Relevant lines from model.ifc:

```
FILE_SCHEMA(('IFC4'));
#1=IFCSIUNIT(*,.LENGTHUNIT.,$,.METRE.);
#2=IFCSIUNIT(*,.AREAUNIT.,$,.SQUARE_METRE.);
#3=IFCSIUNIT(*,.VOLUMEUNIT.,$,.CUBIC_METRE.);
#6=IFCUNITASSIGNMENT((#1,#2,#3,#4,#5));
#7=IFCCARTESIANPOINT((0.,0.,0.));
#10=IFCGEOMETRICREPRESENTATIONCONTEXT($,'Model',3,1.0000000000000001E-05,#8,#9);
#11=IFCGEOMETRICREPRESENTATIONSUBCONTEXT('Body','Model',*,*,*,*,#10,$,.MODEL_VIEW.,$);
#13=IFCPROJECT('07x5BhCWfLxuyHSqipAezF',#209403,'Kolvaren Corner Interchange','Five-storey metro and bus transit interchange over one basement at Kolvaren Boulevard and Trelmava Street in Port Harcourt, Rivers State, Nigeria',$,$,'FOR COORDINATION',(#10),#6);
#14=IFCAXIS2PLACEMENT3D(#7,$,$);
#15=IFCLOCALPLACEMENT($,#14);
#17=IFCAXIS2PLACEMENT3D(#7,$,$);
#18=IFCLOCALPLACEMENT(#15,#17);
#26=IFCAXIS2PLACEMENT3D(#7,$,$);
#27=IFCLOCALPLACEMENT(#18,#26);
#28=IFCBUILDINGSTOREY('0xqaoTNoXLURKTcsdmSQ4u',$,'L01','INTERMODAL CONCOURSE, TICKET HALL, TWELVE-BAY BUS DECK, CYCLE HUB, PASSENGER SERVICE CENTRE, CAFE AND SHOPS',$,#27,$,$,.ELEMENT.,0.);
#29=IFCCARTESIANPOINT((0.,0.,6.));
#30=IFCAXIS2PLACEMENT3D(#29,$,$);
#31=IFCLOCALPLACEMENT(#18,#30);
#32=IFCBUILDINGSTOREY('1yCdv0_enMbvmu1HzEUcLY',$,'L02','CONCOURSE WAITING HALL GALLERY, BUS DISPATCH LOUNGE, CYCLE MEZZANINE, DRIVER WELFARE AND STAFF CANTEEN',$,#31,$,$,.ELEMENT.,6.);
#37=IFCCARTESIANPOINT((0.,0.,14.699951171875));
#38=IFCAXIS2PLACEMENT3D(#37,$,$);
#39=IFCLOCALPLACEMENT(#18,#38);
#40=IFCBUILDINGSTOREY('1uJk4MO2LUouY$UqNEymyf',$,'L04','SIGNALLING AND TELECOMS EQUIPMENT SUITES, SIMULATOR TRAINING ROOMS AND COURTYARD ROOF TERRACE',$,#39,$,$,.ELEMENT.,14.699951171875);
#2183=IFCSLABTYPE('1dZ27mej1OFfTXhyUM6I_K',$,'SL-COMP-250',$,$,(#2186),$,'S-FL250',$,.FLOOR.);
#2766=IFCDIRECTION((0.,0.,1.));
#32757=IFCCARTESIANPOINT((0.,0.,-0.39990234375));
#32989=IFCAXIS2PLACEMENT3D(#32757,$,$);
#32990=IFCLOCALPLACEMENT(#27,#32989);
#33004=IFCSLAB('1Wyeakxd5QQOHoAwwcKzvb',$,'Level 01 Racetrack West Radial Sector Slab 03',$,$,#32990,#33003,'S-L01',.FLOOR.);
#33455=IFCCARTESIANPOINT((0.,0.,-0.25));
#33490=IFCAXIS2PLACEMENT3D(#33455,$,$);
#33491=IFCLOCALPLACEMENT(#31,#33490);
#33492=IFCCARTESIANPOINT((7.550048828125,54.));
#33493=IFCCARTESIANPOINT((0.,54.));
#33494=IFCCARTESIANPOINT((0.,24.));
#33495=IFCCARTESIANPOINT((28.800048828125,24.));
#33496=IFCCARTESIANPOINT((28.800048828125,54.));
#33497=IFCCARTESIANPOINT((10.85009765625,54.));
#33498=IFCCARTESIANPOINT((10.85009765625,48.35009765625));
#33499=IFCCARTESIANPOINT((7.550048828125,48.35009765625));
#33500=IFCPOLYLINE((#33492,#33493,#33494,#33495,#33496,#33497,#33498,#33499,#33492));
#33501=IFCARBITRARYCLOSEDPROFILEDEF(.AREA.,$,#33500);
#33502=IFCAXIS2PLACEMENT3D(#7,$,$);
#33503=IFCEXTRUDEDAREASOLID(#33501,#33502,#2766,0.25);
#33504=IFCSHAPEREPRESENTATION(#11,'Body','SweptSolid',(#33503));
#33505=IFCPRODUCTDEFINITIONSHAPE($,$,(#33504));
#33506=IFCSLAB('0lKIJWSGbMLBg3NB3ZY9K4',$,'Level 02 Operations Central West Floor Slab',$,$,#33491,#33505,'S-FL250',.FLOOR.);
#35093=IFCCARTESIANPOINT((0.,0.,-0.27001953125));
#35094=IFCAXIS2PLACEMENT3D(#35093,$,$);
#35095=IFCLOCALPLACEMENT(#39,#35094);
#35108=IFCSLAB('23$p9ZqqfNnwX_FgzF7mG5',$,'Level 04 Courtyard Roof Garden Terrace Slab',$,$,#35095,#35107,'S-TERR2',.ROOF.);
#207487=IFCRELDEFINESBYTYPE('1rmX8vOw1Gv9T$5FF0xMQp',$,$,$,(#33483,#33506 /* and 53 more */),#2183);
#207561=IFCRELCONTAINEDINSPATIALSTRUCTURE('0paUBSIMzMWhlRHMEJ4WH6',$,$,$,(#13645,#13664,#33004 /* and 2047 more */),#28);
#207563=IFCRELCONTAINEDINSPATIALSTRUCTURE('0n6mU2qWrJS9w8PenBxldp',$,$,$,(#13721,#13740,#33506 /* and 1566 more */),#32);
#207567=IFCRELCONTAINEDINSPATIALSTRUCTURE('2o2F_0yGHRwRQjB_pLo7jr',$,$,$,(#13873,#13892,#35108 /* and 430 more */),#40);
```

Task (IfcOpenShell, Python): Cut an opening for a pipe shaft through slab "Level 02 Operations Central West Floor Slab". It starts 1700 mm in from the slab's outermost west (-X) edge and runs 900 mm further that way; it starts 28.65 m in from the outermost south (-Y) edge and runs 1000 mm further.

```python
import numpy as np
import ifcopenshell
import ifcopenshell.api.feature
import ifcopenshell.api.geometry
import ifcopenshell.api.root
import ifcopenshell.geom
import ifcopenshell.util.placement
import ifcopenshell.util.representation
import ifcopenshell.util.shape
import ifcopenshell.util.unit

model = ifcopenshell.open("model.ifc")
unit_scale = ifcopenshell.util.unit.calculate_unit_scale(model)
settings = ifcopenshell.geom.settings()


def volume(element):
    """Net volume in cubic metres, openings subtracted."""
    shape = ifcopenshell.geom.create_shape(settings, element)
    return ifcopenshell.util.shape.get_volume(shape.geometry)


slab = model.by_id(33506)
before = volume(slab)

# Extent in the slab's own axes, in metres. The edges named are its -X and -Y sides.
slab_shape = ifcopenshell.geom.create_shape(settings, slab)
vertices = ifcopenshell.util.shape.get_vertices(slab_shape.geometry)
x_min, y_min, bottom = vertices.min(axis=0)
top = vertices[:, 2].max()

opening = ifcopenshell.api.root.create_entity(model, ifc_class="IfcOpeningElement", name="Pipe shaft opening", predefined_type="OPENING")
context = ifcopenshell.util.representation.get_context(model, "Model", "Body", "MODEL_VIEW")
width, depth = 0.9, 1
outline = [(0.0, 0.0), (width, 0.0), (width, depth), (0.0, depth), (0.0, 0.0)]
# Overshoot both faces by 50 mm so the cut is clean.
shape = ifcopenshell.api.geometry.add_slab_representation(
    model, context=context, depth=top - bottom + 0.1, polyline=outline
)
ifcopenshell.api.geometry.assign_representation(model, product=opening, representation=shape)

matrix = ifcopenshell.util.placement.get_local_placement(slab.ObjectPlacement)
matrix[:, 3] = matrix @ np.append(np.array([x_min + 1.7, y_min + 28.65, bottom - 0.05]) / unit_scale, 1.0)
ifcopenshell.api.geometry.edit_object_placement(model, product=opening, matrix=matrix, is_si=False)
ifcopenshell.api.feature.add_feature(model, feature=opening, element=slab)

after = volume(slab)

print(f"slab volume {before:.3f} -> {after:.3f} m3")

model.write("model_v2.ifc")
```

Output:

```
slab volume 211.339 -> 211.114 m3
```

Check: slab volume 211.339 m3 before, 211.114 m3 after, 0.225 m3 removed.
